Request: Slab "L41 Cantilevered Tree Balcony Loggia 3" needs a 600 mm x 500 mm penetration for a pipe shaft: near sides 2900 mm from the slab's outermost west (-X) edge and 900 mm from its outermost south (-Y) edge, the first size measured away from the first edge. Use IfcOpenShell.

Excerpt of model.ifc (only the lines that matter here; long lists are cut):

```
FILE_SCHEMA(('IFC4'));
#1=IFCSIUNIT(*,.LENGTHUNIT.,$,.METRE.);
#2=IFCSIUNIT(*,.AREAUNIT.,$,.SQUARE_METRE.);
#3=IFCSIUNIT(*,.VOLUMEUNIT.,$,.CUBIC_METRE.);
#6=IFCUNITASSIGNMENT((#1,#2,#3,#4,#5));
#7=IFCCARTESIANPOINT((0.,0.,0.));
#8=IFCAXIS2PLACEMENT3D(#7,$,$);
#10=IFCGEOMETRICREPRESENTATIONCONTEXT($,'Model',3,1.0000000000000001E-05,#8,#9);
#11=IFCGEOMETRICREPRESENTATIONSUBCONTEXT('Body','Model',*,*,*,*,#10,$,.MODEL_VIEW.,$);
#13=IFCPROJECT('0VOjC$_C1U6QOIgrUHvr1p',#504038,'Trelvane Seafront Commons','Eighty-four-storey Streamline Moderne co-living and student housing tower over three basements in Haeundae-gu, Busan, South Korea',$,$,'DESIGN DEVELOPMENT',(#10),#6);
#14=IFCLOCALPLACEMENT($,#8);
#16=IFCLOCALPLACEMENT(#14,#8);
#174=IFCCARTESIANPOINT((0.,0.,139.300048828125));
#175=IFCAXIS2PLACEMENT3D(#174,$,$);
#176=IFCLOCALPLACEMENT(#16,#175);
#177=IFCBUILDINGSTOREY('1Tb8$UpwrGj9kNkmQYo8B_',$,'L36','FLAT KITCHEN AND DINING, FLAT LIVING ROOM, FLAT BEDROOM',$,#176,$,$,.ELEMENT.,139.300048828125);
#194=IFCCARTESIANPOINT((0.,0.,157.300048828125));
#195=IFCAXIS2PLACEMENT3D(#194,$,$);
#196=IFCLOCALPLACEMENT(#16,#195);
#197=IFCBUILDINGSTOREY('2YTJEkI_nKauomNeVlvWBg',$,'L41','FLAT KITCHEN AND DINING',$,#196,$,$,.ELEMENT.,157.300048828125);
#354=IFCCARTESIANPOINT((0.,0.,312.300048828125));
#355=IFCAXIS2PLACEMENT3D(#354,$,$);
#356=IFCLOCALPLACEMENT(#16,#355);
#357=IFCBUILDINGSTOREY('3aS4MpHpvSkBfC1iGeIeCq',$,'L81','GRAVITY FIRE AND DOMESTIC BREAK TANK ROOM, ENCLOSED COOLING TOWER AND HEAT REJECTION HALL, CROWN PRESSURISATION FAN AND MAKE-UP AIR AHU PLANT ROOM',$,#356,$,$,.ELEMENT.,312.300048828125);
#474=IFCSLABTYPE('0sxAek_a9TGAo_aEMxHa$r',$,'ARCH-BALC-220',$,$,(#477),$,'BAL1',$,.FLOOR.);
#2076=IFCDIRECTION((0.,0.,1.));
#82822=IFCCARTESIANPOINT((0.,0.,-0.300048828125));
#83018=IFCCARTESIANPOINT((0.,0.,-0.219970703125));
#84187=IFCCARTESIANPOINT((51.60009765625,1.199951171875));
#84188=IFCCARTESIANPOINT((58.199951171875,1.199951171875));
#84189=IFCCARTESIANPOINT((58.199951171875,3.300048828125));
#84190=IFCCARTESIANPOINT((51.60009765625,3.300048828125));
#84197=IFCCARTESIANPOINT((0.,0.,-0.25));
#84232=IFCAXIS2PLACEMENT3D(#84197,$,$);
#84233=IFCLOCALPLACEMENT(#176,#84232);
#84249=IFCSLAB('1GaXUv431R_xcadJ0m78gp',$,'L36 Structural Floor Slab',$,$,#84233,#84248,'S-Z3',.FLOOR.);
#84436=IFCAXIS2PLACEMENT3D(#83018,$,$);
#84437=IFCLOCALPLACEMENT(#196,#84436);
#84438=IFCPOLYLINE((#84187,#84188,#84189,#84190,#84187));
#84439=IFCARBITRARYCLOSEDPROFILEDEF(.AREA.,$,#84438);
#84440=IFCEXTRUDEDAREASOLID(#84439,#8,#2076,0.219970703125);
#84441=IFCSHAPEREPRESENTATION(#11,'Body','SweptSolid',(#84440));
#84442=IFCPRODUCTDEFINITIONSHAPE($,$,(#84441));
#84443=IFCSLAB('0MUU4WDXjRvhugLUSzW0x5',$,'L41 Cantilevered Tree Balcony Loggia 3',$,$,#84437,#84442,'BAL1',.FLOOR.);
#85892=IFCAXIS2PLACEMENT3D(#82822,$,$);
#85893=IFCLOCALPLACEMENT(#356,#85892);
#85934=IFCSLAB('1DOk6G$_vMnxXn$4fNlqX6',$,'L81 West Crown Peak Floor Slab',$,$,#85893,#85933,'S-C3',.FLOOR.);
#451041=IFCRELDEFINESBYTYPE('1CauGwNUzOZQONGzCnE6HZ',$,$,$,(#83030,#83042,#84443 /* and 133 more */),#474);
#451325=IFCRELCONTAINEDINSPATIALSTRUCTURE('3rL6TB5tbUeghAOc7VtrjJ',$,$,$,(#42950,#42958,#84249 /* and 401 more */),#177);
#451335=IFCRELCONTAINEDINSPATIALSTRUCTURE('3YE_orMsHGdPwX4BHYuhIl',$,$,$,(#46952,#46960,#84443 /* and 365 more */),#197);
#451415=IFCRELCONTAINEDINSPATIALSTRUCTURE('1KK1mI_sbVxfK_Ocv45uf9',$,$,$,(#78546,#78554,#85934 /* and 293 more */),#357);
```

```python
import numpy as np
import ifcopenshell
import ifcopenshell.api.feature
import ifcopenshell.api.geometry
import ifcopenshell.api.root
import ifcopenshell.geom
import ifcopenshell.util.placement
import ifcopenshell.util.representation
import ifcopenshell.util.shape
import ifcopenshell.util.unit

model = ifcopenshell.open("model.ifc")
unit_scale = ifcopenshell.util.unit.calculate_unit_scale(model)
settings = ifcopenshell.geom.settings()


def volume(element):
    """Net volume in cubic metres, openings subtracted."""
    shape = ifcopenshell.geom.create_shape(settings, element)
    return ifcopenshell.util.shape.get_volume(shape.geometry)


slab = model.by_id(84443)
before = volume(slab)

# Extent in the slab's own axes, in metres. The edges named are its -X and -Y sides.
slab_shape = ifcopenshell.geom.create_shape(settings, slab)
vertices = ifcopenshell.util.shape.get_vertices(slab_shape.geometry)
x_min, y_min, bottom = vertices.min(axis=0)
top = vertices[:, 2].max()

opening = ifcopenshell.api.root.create_entity(model, ifc_class="IfcOpeningElement", name="Pipe shaft opening", predefined_type="OPENING")
context = ifcopenshell.util.representation.get_context(model, "Model", "Body", "MODEL_VIEW")
width, depth = 0.6, 0.5
outline = [(0.0, 0.0), (width, 0.0), (width, depth), (0.0, depth), (0.0, 0.0)]
# Overshoot both faces by 50 mm so the cut is clean.
shape = ifcopenshell.api.geometry.add_slab_representation(
    model, context=context, depth=top - bottom + 0.1, polyline=outline
)
ifcopenshell.api.geometry.assign_representation(model, product=opening, representation=shape)

matrix = ifcopenshell.util.placement.get_local_placement(slab.ObjectPlacement)
matrix[:, 3] = matrix @ np.append(np.array([x_min + 2.9, y_min + 0.9, bottom - 0.05]) / unit_scale, 1.0)
ifcopenshell.api.geometry.edit_object_placement(model, product=opening, matrix=matrix, is_si=False)
ifcopenshell.api.feature.add_feature(model, feature=opening, element=slab)

after = volume(slab)

print(f"slab volume {before:.3f} -> {after:.3f} m3")

model.write("model_v2.ifc")
```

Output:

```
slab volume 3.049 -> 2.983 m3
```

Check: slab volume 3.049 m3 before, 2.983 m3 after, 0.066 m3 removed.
